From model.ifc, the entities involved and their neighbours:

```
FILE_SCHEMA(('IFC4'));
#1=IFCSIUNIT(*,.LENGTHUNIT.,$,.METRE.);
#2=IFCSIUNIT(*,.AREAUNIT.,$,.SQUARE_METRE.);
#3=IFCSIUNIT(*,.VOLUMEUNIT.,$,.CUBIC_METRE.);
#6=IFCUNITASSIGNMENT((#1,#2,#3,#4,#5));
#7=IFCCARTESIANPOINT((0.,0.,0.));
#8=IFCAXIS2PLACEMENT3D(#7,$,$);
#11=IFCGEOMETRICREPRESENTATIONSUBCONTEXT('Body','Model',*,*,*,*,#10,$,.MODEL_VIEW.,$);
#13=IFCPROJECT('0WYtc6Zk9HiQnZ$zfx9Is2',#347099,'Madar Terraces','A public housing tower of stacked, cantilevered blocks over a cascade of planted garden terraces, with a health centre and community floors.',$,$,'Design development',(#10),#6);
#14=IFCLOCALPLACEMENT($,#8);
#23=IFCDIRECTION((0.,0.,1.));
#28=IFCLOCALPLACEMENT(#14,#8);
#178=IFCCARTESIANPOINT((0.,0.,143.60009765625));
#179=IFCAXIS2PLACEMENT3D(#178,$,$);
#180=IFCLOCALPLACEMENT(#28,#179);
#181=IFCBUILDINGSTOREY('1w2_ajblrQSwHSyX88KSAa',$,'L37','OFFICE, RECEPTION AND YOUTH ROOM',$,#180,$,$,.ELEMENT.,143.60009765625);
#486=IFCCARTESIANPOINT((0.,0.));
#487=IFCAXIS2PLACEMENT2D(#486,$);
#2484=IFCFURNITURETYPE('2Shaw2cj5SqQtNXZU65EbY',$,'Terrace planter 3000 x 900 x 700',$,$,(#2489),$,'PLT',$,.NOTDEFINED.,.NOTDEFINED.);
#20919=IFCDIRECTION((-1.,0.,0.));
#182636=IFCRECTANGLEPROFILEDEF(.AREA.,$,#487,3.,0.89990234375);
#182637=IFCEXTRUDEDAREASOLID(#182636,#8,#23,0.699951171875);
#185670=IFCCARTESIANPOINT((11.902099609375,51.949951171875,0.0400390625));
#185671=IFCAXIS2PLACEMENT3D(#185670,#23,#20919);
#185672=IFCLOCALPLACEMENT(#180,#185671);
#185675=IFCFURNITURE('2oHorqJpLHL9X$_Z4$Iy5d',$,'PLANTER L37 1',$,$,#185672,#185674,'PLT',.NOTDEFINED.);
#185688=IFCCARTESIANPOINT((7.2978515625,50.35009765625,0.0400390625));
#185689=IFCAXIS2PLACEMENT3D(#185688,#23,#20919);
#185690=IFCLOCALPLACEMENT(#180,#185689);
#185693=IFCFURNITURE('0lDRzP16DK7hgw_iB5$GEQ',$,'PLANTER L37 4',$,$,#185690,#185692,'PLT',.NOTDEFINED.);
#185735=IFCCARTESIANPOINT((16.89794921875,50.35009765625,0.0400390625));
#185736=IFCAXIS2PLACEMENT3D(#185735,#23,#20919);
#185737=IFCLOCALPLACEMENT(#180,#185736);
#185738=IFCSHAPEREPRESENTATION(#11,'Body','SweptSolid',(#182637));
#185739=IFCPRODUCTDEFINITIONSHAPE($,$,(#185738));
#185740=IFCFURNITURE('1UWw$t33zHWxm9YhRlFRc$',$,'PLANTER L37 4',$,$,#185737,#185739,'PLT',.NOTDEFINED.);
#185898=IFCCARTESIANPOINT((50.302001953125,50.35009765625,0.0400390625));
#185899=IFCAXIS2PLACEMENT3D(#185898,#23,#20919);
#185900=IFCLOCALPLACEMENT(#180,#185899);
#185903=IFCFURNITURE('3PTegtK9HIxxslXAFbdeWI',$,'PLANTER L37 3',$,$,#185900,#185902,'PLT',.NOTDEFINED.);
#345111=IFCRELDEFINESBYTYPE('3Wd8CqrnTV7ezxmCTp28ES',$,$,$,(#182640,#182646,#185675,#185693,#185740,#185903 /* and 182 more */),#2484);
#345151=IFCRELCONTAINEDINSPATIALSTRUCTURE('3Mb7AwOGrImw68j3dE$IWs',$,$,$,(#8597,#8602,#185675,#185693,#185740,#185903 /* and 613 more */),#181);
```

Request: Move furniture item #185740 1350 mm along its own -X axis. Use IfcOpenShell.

```python
import ifcopenshell
import ifcopenshell.api.geometry
import ifcopenshell.util.placement
import ifcopenshell.util.unit

model = ifcopenshell.open("model.ifc")
unit_scale = ifcopenshell.util.unit.calculate_unit_scale(model)

item = model.by_guid("1UWw$t33zHWxm9YhRlFRc$")
matrix = ifcopenshell.util.placement.get_local_placement(item.ObjectPlacement)
matrix[:3, 3] -= matrix[:3, 0] * 1.35 / unit_scale
ifcopenshell.api.geometry.edit_object_placement(model, product=item, matrix=matrix, is_si=False)

print(ifcopenshell.util.placement.get_local_placement(item.ObjectPlacement).round(3) + 0.0)

model.write("model_edited.ifc")
```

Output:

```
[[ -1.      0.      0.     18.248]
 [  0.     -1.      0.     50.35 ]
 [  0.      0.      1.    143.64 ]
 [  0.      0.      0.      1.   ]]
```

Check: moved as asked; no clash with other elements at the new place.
